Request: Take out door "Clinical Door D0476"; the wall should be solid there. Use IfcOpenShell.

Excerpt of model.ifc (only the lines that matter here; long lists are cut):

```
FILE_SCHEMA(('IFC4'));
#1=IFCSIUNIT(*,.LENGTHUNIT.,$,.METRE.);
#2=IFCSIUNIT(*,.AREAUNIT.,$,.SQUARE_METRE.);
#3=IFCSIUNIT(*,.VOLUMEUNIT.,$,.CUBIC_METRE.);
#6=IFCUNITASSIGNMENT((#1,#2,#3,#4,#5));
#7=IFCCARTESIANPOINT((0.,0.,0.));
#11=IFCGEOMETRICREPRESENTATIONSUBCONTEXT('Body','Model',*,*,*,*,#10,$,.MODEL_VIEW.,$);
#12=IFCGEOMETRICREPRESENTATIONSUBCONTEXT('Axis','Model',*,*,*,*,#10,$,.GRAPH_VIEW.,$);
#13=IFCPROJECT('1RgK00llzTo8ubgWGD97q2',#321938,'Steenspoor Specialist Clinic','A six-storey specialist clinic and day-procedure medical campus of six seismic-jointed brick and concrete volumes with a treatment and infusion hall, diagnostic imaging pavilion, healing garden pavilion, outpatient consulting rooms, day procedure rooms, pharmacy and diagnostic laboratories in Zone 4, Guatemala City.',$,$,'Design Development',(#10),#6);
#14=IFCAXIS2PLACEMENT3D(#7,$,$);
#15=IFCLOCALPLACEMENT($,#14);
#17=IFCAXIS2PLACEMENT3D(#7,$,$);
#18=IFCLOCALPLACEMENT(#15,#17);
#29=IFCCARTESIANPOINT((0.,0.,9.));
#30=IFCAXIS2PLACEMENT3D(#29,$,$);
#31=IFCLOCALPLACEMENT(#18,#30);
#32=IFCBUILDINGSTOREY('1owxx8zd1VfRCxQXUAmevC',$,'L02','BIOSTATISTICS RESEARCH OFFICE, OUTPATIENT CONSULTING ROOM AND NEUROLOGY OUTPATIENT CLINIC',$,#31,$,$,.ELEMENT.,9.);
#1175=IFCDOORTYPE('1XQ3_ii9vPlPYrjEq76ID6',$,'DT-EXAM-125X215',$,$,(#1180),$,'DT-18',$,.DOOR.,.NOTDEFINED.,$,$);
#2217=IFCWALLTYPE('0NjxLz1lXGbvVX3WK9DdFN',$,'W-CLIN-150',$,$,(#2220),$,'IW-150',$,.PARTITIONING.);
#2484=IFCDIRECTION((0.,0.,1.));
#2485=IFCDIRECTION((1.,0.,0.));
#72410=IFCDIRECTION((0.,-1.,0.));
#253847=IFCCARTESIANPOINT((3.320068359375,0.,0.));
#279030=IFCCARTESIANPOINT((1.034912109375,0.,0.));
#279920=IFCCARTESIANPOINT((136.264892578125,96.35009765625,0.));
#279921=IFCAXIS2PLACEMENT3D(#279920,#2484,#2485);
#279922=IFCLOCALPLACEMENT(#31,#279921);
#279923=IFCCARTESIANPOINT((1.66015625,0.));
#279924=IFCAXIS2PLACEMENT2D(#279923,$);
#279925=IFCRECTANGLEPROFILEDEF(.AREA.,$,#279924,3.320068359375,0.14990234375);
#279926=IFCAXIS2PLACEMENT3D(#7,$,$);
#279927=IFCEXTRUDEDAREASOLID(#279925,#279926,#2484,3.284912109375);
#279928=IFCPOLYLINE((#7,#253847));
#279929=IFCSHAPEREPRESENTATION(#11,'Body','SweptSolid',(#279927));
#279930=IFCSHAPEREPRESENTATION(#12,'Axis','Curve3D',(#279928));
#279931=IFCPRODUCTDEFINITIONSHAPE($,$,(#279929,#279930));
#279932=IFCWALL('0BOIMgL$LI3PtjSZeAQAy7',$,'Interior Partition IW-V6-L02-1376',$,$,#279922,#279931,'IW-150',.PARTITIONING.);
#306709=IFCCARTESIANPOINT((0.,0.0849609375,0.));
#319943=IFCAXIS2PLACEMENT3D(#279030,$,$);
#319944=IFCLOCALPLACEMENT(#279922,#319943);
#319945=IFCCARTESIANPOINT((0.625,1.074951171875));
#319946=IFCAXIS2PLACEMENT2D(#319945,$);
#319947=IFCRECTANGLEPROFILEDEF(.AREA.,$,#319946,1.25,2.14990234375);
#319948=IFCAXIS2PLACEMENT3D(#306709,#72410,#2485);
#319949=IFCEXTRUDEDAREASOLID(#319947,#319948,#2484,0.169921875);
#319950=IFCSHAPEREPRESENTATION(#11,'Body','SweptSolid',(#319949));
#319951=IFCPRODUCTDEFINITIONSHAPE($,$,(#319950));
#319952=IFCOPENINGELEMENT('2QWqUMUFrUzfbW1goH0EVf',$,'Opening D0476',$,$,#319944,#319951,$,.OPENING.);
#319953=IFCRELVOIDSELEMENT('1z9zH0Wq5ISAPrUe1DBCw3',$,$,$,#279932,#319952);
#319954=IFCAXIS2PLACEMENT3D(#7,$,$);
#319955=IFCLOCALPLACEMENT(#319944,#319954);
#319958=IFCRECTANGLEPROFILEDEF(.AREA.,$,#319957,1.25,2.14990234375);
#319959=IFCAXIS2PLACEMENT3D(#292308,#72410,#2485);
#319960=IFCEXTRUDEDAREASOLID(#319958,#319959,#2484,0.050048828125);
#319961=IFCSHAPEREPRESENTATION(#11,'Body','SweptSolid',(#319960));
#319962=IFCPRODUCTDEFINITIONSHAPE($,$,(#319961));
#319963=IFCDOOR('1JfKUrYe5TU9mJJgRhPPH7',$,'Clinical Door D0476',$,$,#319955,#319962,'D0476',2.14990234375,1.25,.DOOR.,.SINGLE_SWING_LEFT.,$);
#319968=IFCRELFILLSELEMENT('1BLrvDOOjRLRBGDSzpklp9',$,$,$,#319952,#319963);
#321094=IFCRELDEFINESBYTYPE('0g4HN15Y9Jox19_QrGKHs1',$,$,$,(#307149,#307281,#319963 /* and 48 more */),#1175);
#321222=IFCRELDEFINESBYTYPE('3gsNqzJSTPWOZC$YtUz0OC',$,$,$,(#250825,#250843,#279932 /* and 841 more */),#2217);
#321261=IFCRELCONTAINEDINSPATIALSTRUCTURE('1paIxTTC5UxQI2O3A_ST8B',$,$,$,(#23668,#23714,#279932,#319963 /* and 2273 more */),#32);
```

```python
import ifcopenshell
import ifcopenshell.api.feature
import ifcopenshell.api.root
import ifcopenshell.geom
import ifcopenshell.util.shape

model = ifcopenshell.open("model.ifc")
settings = ifcopenshell.geom.settings()


def volume(element):
    """Net volume in cubic metres, openings subtracted."""
    shape = ifcopenshell.geom.create_shape(settings, element)
    return ifcopenshell.util.shape.get_volume(shape.geometry)


door = model.by_guid("1JfKUrYe5TU9mJJgRhPPH7")
opening = door.FillsVoids[0].RelatingOpeningElement
wall = opening.VoidsElements[0].RelatingBuildingElement
before = volume(wall)

ifcopenshell.api.root.remove_product(model, product=door)
ifcopenshell.api.feature.remove_feature(model, feature=opening)

after = volume(wall)

print(f"wall volume {before:.3f} -> {after:.3f} m3")

model.write("model_edited.ifc")
```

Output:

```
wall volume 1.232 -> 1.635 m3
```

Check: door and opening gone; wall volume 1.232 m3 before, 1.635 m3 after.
